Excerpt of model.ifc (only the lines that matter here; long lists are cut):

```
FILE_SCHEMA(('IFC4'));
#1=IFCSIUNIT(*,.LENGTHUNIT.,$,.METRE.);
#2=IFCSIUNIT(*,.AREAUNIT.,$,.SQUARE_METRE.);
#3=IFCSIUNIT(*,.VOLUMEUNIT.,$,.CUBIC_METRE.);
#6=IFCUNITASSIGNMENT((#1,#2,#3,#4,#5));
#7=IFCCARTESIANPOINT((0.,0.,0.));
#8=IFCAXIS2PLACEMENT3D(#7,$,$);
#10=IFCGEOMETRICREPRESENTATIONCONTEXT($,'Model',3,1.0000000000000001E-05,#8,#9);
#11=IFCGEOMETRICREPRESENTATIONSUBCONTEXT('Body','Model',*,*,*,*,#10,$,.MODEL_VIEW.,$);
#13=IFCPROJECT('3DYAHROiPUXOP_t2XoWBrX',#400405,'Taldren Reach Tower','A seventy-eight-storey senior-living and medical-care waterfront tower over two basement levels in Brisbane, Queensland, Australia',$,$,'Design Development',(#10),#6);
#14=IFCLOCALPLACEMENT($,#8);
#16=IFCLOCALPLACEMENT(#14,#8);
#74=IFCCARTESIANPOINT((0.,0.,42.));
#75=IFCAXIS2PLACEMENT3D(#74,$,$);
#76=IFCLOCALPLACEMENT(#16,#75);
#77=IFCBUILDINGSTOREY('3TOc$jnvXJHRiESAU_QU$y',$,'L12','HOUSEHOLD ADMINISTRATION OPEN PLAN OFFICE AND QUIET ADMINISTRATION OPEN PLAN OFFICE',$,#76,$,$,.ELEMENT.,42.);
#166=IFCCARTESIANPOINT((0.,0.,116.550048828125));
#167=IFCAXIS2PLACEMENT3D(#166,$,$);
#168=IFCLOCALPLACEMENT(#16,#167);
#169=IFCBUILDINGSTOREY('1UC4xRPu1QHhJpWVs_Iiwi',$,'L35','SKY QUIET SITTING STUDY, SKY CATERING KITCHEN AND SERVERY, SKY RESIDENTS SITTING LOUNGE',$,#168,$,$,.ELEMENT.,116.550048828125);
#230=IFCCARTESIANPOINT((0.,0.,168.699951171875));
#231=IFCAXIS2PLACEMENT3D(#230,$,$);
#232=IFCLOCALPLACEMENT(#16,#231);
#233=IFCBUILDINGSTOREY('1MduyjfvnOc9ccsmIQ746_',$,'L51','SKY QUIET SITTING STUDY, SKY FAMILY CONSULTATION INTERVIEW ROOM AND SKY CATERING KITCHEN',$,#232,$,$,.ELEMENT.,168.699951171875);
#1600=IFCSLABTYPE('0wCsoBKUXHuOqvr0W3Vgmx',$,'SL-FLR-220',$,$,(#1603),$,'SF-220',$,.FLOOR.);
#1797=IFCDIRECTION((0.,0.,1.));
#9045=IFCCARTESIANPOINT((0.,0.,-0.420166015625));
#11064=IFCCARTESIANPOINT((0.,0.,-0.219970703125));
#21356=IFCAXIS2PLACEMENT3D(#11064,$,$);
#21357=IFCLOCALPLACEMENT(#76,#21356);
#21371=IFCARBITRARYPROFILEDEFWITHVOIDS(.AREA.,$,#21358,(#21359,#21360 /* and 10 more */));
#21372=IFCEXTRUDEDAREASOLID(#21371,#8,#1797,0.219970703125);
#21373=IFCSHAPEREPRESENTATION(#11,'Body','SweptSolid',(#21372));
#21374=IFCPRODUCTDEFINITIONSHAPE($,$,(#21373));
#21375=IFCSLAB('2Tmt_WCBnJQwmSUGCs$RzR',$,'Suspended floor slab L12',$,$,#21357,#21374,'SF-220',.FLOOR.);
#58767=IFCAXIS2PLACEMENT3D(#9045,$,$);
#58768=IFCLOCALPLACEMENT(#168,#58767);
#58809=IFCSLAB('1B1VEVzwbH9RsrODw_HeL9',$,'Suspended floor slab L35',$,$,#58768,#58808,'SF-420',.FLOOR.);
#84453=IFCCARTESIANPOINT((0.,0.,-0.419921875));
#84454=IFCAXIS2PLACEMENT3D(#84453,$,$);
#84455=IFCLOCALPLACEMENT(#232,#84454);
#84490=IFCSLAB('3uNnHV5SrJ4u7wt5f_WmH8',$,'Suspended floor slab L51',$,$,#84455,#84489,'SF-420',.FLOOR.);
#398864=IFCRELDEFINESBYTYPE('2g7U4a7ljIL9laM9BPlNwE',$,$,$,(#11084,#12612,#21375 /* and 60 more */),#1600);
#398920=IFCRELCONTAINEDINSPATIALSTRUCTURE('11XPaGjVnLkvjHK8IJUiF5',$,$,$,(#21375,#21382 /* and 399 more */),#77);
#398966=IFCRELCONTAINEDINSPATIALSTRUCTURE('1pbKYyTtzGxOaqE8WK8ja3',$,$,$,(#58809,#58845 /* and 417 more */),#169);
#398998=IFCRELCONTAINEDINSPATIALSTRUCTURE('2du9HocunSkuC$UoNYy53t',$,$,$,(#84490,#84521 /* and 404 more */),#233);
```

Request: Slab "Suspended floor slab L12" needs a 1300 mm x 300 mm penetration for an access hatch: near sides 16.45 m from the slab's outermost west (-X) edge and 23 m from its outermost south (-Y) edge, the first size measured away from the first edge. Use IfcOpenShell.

```python
import numpy as np
import ifcopenshell
import ifcopenshell.api.feature
import ifcopenshell.api.geometry
import ifcopenshell.api.root
import ifcopenshell.geom
import ifcopenshell.util.placement
import ifcopenshell.util.representation
import ifcopenshell.util.shape
import ifcopenshell.util.unit

model = ifcopenshell.open("model.ifc")
unit_scale = ifcopenshell.util.unit.calculate_unit_scale(model)
settings = ifcopenshell.geom.settings()


def volume(element):
    """Net volume in cubic metres, openings subtracted."""
    shape = ifcopenshell.geom.create_shape(settings, element)
    return ifcopenshell.util.shape.get_volume(shape.geometry)


slab = model.by_id(21375)
before = volume(slab)

# Extent in the slab's own axes, in metres. The edges named are its -X and -Y sides.
slab_shape = ifcopenshell.geom.create_shape(settings, slab)
vertices = ifcopenshell.util.shape.get_vertices(slab_shape.geometry)
x_min, y_min, bottom = vertices.min(axis=0)
top = vertices[:, 2].max()

opening = ifcopenshell.api.root.create_entity(model, ifc_class="IfcOpeningElement", name="Access hatch opening", predefined_type="OPENING")
context = ifcopenshell.util.representation.get_context(model, "Model", "Body", "MODEL_VIEW")
width, depth = 1.3, 0.3
outline = [(0.0, 0.0), (width, 0.0), (width, depth), (0.0, depth), (0.0, 0.0)]
# Overshoot both faces by 50 mm so the cut is clean.
shape = ifcopenshell.api.geometry.add_slab_representation(
    model, context=context, depth=top - bottom + 0.1, polyline=outline
)
ifcopenshell.api.geometry.assign_representation(model, product=opening, representation=shape)

matrix = ifcopenshell.util.placement.get_local_placement(slab.ObjectPlacement)
matrix[:, 3] = matrix @ np.append(np.array([x_min + 16.45, y_min + 23, bottom - 0.05]) / unit_scale, 1.0)
ifcopenshell.api.geometry.edit_object_placement(model, product=opening, matrix=matrix, is_si=False)
ifcopenshell.api.feature.add_feature(model, feature=opening, element=slab)

after = volume(slab)

print(f"slab volume {before:.3f} -> {after:.3f} m3")

model.write("model-out.ifc")
```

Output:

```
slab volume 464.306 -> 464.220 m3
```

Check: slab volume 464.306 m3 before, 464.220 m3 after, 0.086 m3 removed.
